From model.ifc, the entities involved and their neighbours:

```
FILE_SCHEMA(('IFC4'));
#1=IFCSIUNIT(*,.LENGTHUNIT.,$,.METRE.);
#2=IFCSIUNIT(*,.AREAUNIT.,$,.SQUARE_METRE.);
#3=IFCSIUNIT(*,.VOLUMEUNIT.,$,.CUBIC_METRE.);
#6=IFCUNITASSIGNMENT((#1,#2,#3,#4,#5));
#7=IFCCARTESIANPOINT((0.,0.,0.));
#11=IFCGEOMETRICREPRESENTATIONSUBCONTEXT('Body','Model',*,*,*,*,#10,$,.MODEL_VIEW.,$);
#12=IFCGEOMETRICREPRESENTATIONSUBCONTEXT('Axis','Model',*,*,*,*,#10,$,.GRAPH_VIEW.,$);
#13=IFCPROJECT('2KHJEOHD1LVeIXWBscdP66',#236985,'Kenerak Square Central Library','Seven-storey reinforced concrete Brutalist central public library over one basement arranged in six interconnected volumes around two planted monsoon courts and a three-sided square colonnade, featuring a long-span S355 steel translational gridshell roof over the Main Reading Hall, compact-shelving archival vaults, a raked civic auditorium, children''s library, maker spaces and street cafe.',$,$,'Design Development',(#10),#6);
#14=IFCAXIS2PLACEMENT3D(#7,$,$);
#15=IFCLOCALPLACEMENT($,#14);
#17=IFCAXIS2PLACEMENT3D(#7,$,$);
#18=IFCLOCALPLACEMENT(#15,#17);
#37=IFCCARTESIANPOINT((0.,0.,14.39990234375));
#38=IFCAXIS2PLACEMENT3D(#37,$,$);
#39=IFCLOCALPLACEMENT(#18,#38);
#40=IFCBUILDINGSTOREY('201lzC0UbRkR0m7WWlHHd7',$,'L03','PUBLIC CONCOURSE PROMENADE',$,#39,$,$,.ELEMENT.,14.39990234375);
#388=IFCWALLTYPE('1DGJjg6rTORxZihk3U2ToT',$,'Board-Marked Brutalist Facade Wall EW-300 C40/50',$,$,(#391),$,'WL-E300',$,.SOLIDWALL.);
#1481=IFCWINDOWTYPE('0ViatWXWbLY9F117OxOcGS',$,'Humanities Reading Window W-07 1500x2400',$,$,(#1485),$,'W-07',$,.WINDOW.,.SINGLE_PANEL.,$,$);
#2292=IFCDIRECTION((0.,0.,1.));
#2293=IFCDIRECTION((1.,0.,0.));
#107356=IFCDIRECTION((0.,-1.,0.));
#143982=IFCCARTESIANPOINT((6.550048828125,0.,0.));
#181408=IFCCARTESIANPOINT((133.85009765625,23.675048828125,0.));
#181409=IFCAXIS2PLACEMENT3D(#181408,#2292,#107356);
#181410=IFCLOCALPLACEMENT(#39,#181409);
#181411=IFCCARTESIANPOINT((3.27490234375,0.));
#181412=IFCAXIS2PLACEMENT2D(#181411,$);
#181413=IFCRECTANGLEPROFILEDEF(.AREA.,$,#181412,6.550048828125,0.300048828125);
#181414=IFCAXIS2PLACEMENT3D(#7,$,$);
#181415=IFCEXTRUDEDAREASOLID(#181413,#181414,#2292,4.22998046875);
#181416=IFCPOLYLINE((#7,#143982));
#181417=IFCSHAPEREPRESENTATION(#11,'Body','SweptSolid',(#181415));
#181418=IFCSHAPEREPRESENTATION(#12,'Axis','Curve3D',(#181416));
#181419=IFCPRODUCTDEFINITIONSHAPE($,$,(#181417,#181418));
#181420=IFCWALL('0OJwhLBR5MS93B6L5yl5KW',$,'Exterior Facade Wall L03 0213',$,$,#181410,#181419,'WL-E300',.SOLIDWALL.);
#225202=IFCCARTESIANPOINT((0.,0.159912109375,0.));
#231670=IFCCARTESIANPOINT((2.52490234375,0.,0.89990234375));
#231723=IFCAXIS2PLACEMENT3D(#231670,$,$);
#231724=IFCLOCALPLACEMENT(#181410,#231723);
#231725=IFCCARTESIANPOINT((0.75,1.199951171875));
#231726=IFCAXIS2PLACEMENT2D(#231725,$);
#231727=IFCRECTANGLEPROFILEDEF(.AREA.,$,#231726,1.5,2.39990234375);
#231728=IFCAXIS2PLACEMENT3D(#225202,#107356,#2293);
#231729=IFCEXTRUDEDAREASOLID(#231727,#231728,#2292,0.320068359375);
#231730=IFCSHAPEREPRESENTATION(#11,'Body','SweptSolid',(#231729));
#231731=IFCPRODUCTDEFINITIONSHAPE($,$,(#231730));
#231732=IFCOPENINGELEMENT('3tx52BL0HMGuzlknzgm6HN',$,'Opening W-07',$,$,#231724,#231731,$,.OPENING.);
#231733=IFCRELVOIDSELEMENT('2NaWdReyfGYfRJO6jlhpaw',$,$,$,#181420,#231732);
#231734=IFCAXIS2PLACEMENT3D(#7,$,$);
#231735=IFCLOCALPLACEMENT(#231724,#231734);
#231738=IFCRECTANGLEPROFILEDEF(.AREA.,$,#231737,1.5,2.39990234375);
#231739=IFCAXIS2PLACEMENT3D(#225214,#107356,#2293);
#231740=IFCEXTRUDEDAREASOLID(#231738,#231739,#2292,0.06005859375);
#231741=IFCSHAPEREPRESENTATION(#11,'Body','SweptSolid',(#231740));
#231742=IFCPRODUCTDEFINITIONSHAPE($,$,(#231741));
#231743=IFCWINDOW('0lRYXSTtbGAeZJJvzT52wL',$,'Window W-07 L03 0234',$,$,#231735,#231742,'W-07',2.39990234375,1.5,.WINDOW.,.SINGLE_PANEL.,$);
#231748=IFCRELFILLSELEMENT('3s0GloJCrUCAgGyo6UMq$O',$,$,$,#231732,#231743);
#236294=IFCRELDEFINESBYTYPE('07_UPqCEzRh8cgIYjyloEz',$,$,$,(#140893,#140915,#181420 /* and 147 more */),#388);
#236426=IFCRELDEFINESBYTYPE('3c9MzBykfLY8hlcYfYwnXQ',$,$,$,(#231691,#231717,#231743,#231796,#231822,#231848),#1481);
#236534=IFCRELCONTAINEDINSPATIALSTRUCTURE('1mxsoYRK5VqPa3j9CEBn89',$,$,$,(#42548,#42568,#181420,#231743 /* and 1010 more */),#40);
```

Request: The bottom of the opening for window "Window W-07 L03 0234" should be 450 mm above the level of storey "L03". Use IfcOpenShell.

```python
import numpy as np
import ifcopenshell
import ifcopenshell.api.geometry
import ifcopenshell.geom
import ifcopenshell.util.element
import ifcopenshell.util.placement
import ifcopenshell.util.shape
import ifcopenshell.util.unit

model = ifcopenshell.open("model.ifc")
unit_scale = ifcopenshell.util.unit.calculate_unit_scale(model)

window = model.by_id(231743)
opening = window.FillsVoids[0].RelatingOpeningElement
storey = ifcopenshell.util.element.get_container(window, ifc_class="IfcBuildingStorey")
level = ifcopenshell.util.placement.get_local_placement(storey.ObjectPlacement)[2, 3]

# The opening's origin need not be at the sill, so measure its lowest point.
shape = ifcopenshell.geom.create_shape(ifcopenshell.geom.settings(), opening)
bottom = ifcopenshell.util.shape.get_shape_bottom_elevation(shape, shape.geometry) / unit_scale
dz = level + 0.45 / unit_scale - bottom

shift = np.array([0.0, 0.0, dz])
# The window is placed relative to its opening, so it follows when the opening moves.
matrix = ifcopenshell.util.placement.get_local_placement(opening.ObjectPlacement)
matrix[:3, 3] += shift
ifcopenshell.api.geometry.edit_object_placement(
    model, product=opening, matrix=matrix, is_si=False, should_transform_children=True
)

print(f"moved by {dz * unit_scale:+.3f} m")

model.write("model_rev.ifc")
```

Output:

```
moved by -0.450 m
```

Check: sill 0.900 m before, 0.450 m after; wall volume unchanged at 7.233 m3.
